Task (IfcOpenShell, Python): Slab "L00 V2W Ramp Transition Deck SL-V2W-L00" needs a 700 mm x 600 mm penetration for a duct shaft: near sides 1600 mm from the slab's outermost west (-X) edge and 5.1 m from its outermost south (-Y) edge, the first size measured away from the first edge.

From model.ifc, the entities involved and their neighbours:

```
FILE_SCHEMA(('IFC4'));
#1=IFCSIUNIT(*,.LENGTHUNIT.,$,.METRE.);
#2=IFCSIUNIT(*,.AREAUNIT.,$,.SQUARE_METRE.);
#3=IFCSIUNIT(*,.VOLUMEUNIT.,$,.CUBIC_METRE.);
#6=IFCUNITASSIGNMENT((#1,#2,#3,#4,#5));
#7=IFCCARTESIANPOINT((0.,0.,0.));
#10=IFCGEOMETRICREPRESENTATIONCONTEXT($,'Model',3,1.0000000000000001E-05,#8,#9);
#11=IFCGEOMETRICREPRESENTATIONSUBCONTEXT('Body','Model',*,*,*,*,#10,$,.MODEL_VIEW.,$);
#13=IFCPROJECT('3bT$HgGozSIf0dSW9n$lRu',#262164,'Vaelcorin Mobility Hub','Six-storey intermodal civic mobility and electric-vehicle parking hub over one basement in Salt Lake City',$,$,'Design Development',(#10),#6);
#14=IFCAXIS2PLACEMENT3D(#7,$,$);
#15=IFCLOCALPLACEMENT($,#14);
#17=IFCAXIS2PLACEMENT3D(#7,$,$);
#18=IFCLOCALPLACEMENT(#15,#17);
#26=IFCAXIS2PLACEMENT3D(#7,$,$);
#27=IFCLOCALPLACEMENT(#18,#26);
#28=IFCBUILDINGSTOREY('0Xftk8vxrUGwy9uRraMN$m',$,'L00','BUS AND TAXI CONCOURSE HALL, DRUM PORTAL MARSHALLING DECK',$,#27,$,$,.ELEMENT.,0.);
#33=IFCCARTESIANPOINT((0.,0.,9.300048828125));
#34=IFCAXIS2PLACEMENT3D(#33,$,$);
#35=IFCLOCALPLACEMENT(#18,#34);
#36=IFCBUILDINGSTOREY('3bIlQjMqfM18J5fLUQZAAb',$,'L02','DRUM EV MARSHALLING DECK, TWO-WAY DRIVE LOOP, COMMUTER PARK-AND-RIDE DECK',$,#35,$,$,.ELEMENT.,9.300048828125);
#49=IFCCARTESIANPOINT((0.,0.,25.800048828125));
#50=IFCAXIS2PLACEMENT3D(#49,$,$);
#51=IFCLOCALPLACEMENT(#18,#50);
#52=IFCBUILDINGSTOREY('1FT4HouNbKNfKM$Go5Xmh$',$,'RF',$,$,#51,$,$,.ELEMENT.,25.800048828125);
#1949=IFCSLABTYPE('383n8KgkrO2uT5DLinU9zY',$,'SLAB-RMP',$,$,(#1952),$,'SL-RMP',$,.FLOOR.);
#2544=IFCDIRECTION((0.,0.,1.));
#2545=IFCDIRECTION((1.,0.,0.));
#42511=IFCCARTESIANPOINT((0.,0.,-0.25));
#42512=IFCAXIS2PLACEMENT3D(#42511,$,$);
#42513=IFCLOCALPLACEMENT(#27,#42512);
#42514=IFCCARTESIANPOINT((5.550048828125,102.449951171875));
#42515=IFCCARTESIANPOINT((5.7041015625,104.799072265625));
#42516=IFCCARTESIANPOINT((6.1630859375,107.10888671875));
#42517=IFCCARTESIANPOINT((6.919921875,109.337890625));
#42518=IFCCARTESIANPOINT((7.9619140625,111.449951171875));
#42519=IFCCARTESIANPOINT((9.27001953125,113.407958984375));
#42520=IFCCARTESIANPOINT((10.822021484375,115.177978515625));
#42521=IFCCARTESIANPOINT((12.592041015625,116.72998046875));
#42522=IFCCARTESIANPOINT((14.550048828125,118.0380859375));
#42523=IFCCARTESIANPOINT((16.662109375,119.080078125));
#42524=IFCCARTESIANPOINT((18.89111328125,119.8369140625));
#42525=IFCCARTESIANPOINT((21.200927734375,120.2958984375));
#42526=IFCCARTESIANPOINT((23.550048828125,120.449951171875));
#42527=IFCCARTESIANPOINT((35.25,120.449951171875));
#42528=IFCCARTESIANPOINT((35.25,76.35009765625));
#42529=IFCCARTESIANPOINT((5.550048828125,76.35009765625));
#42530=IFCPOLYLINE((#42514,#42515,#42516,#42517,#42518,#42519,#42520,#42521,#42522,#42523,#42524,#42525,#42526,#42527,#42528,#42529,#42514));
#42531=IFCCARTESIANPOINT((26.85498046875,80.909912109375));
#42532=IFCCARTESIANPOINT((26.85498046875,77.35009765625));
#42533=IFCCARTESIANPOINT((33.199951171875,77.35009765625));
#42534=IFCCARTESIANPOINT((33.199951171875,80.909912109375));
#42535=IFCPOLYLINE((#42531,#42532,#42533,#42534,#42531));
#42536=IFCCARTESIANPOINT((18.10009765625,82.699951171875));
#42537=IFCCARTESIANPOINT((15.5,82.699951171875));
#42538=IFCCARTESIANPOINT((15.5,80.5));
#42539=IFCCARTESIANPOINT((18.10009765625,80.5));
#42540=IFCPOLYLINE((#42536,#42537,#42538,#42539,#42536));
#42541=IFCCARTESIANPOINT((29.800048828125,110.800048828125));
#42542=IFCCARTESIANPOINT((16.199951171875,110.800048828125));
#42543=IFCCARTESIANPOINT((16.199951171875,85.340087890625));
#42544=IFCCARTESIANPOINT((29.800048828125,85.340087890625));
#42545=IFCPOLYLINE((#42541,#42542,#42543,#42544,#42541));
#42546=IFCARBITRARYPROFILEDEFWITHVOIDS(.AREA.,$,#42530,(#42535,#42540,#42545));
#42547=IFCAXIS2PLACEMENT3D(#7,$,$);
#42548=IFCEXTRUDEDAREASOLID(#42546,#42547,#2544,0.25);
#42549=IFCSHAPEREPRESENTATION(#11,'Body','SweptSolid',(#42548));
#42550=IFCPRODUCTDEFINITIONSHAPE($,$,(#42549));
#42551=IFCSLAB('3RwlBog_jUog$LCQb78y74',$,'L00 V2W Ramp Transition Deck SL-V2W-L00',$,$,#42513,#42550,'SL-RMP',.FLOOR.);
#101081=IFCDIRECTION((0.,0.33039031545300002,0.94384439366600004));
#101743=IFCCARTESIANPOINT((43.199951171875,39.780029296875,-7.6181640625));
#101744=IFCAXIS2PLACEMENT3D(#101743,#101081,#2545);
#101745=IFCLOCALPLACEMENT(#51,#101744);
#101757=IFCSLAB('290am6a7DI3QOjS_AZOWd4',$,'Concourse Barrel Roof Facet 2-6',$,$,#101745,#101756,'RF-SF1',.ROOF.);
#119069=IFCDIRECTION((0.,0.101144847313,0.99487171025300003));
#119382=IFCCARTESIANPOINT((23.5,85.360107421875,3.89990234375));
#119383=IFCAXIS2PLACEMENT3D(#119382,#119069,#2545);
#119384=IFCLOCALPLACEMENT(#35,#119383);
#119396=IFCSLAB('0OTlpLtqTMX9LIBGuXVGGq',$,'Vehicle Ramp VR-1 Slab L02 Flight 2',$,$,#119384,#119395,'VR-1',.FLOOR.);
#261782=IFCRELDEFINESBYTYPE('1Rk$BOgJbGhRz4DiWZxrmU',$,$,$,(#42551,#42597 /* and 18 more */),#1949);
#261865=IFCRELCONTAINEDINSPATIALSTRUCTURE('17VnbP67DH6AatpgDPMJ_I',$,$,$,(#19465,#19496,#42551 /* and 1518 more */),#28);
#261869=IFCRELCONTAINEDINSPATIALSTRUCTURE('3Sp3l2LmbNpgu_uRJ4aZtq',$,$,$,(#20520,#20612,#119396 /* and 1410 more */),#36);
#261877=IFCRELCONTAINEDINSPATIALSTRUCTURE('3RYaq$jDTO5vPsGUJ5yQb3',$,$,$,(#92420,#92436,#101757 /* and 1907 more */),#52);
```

```python
import numpy as np
import ifcopenshell
import ifcopenshell.api.feature
import ifcopenshell.api.geometry
import ifcopenshell.api.root
import ifcopenshell.geom
import ifcopenshell.util.placement
import ifcopenshell.util.representation
import ifcopenshell.util.shape
import ifcopenshell.util.unit

model = ifcopenshell.open("model.ifc")
unit_scale = ifcopenshell.util.unit.calculate_unit_scale(model)
settings = ifcopenshell.geom.settings()


def volume(element):
    """Net volume in cubic metres, openings subtracted."""
    shape = ifcopenshell.geom.create_shape(settings, element)
    return ifcopenshell.util.shape.get_volume(shape.geometry)


slab = model.by_guid("3RwlBog_jUog$LCQb78y74")
before = volume(slab)

# Extent in the slab's own axes, in metres. The edges named are its -X and -Y sides.
slab_shape = ifcopenshell.geom.create_shape(settings, slab)
vertices = ifcopenshell.util.shape.get_vertices(slab_shape.geometry)
x_min, y_min, bottom = vertices.min(axis=0)
top = vertices[:, 2].max()

opening = ifcopenshell.api.root.create_entity(model, ifc_class="IfcOpeningElement", name="Duct shaft opening", predefined_type="OPENING")
context = ifcopenshell.util.representation.get_context(model, "Model", "Body", "MODEL_VIEW")
width, depth = 0.7, 0.6
outline = [(0.0, 0.0), (width, 0.0), (width, depth), (0.0, depth), (0.0, 0.0)]
# Overshoot both faces by 50 mm so the cut is clean.
shape = ifcopenshell.api.geometry.add_slab_representation(
    model, context=context, depth=top - bottom + 0.1, polyline=outline
)
ifcopenshell.api.geometry.assign_representation(model, product=opening, representation=shape)

matrix = ifcopenshell.util.placement.get_local_placement(slab.ObjectPlacement)
matrix[:, 3] = matrix @ np.append(np.array([x_min + 1.6, y_min + 5.1, bottom - 0.05]) / unit_scale, 1.0)
ifcopenshell.api.geometry.edit_object_placement(model, product=opening, matrix=matrix, is_si=False)
ifcopenshell.api.feature.add_feature(model, feature=opening, element=slab)

after = volume(slab)

print(f"slab volume {before:.3f} -> {after:.3f} m3")

model.write("model_edited.ifc")
```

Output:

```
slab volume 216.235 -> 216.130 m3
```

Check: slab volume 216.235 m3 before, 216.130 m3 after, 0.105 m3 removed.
